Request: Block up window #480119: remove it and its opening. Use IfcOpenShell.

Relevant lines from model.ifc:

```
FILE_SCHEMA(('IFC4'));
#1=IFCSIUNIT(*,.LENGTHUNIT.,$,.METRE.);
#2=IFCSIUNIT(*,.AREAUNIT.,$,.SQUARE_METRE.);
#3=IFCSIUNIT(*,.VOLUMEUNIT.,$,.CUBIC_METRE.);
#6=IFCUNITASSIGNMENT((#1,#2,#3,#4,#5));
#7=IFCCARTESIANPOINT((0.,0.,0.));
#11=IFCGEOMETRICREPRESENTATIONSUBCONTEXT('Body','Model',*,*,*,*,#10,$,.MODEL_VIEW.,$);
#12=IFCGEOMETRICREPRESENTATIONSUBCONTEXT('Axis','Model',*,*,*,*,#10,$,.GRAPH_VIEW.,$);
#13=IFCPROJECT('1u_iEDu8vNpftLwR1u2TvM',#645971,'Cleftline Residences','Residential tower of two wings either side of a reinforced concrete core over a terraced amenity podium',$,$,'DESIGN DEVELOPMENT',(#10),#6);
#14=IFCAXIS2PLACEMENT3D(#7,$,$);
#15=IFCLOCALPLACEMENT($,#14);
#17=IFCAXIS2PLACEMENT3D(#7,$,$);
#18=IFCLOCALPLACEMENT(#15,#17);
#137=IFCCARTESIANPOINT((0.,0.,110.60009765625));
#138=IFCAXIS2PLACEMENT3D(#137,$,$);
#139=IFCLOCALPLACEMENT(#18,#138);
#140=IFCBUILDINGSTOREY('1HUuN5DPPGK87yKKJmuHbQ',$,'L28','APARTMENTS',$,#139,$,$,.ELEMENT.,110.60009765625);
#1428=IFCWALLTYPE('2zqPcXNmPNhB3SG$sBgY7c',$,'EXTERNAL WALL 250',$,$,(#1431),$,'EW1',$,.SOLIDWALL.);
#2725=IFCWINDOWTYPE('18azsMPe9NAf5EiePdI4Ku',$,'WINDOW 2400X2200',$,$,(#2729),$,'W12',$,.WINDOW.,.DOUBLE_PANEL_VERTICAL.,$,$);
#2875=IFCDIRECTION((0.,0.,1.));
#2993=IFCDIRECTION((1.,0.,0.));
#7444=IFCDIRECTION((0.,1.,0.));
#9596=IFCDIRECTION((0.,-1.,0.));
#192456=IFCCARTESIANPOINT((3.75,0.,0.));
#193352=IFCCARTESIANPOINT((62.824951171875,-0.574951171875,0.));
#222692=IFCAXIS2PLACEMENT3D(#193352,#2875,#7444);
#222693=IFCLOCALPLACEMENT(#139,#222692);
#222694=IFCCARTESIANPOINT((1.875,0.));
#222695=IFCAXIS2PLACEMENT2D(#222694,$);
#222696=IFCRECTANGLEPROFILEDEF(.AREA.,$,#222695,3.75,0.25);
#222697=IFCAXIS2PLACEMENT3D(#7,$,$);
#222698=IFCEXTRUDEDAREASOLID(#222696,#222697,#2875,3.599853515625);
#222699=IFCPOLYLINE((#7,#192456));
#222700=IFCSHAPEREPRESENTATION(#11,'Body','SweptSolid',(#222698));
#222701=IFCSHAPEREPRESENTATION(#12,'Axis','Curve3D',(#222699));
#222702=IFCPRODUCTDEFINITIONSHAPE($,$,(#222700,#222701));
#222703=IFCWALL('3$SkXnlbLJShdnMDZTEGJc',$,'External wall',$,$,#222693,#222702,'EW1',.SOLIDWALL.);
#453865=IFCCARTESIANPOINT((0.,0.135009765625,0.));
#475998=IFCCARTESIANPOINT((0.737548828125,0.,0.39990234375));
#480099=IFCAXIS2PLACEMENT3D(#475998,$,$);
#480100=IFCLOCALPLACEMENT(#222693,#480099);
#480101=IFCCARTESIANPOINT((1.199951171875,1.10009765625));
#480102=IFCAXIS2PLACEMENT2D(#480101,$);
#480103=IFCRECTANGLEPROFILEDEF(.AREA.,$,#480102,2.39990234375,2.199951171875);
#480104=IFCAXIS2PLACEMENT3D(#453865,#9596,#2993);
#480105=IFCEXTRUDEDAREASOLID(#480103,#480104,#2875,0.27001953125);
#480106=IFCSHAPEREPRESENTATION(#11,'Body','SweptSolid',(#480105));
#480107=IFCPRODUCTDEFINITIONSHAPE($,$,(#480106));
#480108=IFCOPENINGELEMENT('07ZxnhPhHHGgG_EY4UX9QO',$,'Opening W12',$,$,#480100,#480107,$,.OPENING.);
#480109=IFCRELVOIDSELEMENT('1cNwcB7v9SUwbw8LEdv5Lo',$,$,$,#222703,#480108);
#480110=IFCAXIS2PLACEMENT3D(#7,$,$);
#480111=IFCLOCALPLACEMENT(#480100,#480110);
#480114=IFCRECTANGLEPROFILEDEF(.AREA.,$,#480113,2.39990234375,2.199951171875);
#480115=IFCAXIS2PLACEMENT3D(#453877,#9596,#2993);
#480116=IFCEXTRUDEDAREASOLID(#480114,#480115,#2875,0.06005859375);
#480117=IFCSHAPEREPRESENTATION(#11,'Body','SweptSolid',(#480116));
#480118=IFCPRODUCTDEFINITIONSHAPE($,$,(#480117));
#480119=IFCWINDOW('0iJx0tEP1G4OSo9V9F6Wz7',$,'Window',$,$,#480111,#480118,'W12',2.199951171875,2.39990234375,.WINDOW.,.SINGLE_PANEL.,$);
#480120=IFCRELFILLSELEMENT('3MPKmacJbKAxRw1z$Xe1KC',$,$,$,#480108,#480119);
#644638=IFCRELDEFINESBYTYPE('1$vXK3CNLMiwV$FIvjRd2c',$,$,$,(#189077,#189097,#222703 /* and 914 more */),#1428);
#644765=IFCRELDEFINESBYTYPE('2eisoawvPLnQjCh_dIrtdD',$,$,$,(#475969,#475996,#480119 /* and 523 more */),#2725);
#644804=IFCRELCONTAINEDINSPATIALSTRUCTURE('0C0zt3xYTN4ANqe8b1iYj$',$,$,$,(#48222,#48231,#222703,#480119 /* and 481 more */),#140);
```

```python
import ifcopenshell
import ifcopenshell.api.feature
import ifcopenshell.api.root
import ifcopenshell.geom
import ifcopenshell.util.shape

model = ifcopenshell.open("model.ifc")
settings = ifcopenshell.geom.settings()


def volume(element):
    """Net volume in cubic metres, openings subtracted."""
    shape = ifcopenshell.geom.create_shape(settings, element)
    return ifcopenshell.util.shape.get_volume(shape.geometry)


window = model.by_id(480119)
opening = window.FillsVoids[0].RelatingOpeningElement
wall = opening.VoidsElements[0].RelatingBuildingElement
before = volume(wall)

ifcopenshell.api.root.remove_product(model, product=window)
ifcopenshell.api.feature.remove_feature(model, feature=opening)

after = volume(wall)

print(f"wall volume {before:.3f} -> {after:.3f} m3")

model.write("model_updated.ifc")
```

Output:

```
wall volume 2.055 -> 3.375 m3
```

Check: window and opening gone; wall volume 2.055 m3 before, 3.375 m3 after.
